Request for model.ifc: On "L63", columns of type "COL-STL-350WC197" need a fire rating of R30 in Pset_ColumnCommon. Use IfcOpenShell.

First a look at what the model holds.

```python
import ifcopenshell
import ifcopenshell.util.element

model = ifcopenshell.open("model.ifc")
print(model.schema)
storey = next(s for s in model.by_type("IfcBuildingStorey") if s.Name == "L63")
columns = [e for e in ifcopenshell.util.element.get_decomposition(storey) if e.is_a("IfcColumn")]
seen = {}
for e in columns:
    element_type = ifcopenshell.util.element.get_type(e)
    key = (element_type.Name if element_type != e and element_type else None, ifcopenshell.util.element.get_pset(e, "Pset_ColumnCommon", "FireRating"))
    seen[key] = seen.get(key, 0) + 1
for (name, value), count in sorted(seen.items(), key=str):
    print(count, "x", name, "|", value)
```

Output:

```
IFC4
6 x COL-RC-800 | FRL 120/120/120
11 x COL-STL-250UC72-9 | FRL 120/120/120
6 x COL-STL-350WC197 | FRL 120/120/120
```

```python
import ifcopenshell
import ifcopenshell.api.pset
import ifcopenshell.util.element

model = ifcopenshell.open("model.ifc")

storey = next(s for s in model.by_type("IfcBuildingStorey") if s.Name == "L63")
columns = [e for e in ifcopenshell.util.element.get_decomposition(storey) if e.is_a("IfcColumn")]

count = 0
for e in columns:
    element_type = ifcopenshell.util.element.get_type(e)
    if element_type in (None, e) or element_type.Name != "COL-STL-350WC197":
        continue
    # add_pset returns the element's existing set when there is one.
    pset = ifcopenshell.api.pset.add_pset(model, product=e, name="Pset_ColumnCommon")
    ifcopenshell.api.pset.edit_pset(model, pset=pset, properties={"FireRating": "R30"})
    count += 1

print(count, "columns updated")

model.write("model_rev.ifc")
```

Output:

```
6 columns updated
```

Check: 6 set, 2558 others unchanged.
